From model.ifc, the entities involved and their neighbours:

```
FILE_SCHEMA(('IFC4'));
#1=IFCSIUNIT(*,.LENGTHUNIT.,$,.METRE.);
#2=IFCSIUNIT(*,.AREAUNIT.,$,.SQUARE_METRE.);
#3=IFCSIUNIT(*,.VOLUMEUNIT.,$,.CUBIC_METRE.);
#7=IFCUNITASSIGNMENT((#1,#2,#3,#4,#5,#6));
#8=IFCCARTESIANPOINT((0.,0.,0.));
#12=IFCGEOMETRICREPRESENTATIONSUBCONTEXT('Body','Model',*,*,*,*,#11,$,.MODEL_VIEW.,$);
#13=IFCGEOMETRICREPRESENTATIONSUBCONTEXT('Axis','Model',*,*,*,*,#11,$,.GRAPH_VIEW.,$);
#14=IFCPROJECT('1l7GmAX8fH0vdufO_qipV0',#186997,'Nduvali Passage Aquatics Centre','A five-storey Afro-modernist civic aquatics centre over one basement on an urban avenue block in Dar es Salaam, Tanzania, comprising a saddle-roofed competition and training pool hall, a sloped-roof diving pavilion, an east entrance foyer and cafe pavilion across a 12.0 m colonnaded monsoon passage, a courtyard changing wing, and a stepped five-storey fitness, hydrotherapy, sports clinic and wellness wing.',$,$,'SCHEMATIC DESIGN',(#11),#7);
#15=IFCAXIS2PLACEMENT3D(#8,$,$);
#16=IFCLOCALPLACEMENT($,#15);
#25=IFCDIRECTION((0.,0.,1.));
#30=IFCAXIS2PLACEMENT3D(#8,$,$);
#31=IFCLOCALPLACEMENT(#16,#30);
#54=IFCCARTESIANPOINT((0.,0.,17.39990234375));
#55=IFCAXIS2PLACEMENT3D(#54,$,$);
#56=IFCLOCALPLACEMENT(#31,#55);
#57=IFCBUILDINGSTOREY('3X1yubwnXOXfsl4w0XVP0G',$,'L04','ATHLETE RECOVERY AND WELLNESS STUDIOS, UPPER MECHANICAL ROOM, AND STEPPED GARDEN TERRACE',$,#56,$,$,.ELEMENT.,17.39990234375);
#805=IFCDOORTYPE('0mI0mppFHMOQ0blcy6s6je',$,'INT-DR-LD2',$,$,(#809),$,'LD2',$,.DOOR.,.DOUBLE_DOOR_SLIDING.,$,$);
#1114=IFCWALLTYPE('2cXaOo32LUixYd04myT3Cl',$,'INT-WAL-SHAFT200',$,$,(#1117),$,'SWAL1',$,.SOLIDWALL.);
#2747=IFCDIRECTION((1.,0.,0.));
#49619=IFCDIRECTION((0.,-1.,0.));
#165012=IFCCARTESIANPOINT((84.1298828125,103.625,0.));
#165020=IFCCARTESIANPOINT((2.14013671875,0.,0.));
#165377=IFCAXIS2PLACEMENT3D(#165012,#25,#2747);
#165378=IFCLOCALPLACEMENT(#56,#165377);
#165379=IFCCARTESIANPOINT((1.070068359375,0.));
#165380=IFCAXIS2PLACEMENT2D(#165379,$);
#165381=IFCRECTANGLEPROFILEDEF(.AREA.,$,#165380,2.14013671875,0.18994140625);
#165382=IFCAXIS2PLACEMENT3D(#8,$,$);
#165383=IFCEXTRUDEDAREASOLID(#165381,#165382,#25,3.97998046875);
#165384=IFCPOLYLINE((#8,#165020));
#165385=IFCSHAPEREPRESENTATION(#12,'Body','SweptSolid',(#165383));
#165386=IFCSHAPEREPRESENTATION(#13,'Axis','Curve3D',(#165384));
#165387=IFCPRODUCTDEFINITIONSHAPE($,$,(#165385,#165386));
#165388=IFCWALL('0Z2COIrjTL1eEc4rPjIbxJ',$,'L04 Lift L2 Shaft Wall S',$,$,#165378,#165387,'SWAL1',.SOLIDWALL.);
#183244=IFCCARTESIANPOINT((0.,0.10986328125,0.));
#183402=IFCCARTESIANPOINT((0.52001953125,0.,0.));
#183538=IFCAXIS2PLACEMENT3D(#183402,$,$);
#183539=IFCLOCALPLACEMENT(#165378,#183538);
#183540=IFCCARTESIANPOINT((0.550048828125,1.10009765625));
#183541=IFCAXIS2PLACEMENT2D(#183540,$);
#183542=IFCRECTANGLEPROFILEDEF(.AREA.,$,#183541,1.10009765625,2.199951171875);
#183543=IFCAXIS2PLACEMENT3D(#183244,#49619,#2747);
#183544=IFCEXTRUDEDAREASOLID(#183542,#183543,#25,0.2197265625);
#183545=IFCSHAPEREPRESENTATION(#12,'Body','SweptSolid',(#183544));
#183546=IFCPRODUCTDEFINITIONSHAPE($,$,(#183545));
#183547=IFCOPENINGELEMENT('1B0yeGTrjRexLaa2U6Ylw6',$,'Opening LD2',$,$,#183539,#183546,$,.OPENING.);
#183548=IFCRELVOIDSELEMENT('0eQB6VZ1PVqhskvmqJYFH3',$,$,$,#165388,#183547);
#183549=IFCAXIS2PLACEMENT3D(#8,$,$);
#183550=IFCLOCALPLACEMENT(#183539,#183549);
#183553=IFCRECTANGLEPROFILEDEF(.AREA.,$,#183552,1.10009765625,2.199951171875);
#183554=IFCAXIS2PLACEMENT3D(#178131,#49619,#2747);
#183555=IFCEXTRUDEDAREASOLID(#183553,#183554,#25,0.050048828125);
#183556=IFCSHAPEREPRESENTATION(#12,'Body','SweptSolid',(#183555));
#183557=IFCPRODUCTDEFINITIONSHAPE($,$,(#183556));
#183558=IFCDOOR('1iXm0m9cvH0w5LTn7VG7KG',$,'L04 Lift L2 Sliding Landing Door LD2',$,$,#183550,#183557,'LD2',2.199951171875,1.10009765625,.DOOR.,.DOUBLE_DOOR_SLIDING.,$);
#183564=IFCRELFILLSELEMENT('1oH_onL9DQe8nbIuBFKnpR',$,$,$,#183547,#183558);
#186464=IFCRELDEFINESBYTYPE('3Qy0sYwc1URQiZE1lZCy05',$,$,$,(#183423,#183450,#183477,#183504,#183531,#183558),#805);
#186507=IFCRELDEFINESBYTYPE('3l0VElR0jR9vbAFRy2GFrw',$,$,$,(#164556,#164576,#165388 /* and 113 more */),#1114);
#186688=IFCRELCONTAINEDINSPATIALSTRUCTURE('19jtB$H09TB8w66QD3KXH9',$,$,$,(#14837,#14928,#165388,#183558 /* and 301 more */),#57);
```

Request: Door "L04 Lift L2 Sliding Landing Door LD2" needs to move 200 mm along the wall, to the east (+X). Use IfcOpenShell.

```python
import ifcopenshell
import ifcopenshell.api.geometry
import ifcopenshell.util.placement
import ifcopenshell.util.unit

model = ifcopenshell.open("model.ifc")
unit_scale = ifcopenshell.util.unit.calculate_unit_scale(model)

door = model.by_guid("1iXm0m9cvH0w5LTn7VG7KG")
opening = door.FillsVoids[0].RelatingOpeningElement
wall = opening.VoidsElements[0].RelatingBuildingElement

wall_matrix = ifcopenshell.util.placement.get_local_placement(wall.ObjectPlacement)
shift = wall_matrix[:3, 0] * 0.2 / unit_scale
before = ifcopenshell.util.placement.get_local_placement(door.ObjectPlacement)[:3, 3].copy()

# The door is placed relative to its opening, so it follows when the opening moves.
matrix = ifcopenshell.util.placement.get_local_placement(opening.ObjectPlacement)
matrix[:3, 3] += shift
ifcopenshell.api.geometry.edit_object_placement(
    model, product=opening, matrix=matrix, is_si=False, should_transform_children=True
)

after = ifcopenshell.util.placement.get_local_placement(door.ObjectPlacement)[:3, 3]
print("door moved by", (after - before).round(3) + 0.0)

model.write("model_rev.ifc")
```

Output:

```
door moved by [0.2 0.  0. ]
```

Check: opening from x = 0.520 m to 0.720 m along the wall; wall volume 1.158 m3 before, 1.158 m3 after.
